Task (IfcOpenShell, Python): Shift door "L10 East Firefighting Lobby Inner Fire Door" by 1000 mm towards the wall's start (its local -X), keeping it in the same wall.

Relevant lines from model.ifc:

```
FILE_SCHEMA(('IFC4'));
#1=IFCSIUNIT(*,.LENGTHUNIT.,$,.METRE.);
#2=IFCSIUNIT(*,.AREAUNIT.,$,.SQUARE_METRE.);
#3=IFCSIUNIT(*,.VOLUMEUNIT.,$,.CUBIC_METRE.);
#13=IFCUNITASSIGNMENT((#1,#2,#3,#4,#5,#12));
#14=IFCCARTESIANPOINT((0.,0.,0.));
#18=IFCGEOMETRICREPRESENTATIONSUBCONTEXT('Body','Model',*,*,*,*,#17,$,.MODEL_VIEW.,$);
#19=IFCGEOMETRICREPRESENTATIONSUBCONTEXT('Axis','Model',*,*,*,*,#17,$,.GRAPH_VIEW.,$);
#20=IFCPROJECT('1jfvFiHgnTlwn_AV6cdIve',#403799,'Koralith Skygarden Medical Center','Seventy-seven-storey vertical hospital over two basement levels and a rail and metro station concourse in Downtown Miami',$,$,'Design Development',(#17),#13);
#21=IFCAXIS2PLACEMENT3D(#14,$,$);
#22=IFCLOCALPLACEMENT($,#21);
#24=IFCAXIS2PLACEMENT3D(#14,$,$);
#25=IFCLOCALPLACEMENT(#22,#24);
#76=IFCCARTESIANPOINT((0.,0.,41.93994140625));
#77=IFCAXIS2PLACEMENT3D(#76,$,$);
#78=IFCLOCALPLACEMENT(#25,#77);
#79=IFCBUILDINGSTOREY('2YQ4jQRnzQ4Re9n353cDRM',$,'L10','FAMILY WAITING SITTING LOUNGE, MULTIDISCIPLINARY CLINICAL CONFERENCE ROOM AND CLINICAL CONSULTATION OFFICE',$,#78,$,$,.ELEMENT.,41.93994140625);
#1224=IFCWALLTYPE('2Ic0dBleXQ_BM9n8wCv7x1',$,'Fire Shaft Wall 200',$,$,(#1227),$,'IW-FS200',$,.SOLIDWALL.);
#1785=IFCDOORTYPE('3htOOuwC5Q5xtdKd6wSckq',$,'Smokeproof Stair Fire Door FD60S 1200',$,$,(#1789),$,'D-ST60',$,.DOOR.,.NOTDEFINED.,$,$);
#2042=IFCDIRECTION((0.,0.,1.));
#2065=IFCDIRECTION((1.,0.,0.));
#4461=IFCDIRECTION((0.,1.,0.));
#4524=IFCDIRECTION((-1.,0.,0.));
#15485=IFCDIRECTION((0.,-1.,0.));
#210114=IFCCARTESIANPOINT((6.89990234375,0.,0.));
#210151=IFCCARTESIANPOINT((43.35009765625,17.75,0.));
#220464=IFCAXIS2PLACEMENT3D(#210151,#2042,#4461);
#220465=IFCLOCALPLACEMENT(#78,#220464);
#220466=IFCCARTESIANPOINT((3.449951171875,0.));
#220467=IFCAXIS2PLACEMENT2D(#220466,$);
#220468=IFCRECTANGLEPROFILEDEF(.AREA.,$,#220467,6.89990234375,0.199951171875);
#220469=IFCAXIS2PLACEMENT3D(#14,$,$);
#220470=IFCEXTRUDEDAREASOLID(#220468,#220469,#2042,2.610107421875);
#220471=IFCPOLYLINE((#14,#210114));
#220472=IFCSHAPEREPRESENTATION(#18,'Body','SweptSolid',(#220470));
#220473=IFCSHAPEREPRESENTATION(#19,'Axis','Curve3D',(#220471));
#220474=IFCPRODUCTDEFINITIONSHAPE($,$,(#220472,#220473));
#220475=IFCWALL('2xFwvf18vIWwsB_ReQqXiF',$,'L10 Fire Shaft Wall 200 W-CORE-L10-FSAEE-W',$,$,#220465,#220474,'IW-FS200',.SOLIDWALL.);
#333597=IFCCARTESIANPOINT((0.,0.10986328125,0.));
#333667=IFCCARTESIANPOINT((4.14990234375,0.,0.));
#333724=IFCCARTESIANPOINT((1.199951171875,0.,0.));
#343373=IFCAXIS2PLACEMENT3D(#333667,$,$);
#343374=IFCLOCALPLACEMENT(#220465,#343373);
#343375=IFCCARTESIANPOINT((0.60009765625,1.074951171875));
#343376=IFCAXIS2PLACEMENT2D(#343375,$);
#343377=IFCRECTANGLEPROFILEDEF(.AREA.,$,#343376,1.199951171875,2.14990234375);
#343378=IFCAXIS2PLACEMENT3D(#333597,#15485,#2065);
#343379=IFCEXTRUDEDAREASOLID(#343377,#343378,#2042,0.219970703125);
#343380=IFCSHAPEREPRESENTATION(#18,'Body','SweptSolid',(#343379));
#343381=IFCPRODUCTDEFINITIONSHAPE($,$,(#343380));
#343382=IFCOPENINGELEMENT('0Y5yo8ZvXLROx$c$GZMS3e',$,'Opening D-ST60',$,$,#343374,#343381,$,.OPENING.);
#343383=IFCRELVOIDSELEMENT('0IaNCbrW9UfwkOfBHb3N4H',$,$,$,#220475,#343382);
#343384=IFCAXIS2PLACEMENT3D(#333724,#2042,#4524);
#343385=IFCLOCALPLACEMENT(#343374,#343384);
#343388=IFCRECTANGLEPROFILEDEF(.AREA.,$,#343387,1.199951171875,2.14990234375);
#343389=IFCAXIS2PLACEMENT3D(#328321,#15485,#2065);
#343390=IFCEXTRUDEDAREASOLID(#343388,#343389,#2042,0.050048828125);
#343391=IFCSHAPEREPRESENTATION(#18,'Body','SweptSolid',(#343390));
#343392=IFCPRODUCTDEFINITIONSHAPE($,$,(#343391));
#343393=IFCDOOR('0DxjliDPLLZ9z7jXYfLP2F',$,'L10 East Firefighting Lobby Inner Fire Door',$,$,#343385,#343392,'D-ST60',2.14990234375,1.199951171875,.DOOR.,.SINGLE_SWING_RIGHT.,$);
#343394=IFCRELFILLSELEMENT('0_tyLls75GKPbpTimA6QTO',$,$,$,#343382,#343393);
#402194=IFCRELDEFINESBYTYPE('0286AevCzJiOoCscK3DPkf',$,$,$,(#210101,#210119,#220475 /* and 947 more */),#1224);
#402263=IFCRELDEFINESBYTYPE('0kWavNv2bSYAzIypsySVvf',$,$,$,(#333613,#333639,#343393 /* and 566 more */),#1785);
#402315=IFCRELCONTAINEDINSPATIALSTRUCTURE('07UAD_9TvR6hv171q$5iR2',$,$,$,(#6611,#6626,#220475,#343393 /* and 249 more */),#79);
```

```python
import ifcopenshell
import ifcopenshell.api.geometry
import ifcopenshell.util.placement

model = ifcopenshell.open("model.ifc")

door = model.by_guid("0DxjliDPLLZ9z7jXYfLP2F")
opening = door.FillsVoids[0].RelatingOpeningElement
wall = opening.VoidsElements[0].RelatingBuildingElement

wall_matrix = ifcopenshell.util.placement.get_local_placement(wall.ObjectPlacement)
shift = wall_matrix[:3, 0] * -1.0
before = ifcopenshell.util.placement.get_local_placement(door.ObjectPlacement)[:3, 3].copy()

# The door is placed relative to its opening, so it follows when the opening moves.
matrix = ifcopenshell.util.placement.get_local_placement(opening.ObjectPlacement)
matrix[:3, 3] += shift
ifcopenshell.api.geometry.edit_object_placement(
    model, product=opening, matrix=matrix, is_si=False, should_transform_children=True
)

after = ifcopenshell.util.placement.get_local_placement(door.ObjectPlacement)[:3, 3]
print("door moved by", (after - before).round(3) + 0.0)

model.write("model_updated.ifc")
```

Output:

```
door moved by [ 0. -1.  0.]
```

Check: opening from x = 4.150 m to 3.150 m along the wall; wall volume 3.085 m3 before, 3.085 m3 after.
